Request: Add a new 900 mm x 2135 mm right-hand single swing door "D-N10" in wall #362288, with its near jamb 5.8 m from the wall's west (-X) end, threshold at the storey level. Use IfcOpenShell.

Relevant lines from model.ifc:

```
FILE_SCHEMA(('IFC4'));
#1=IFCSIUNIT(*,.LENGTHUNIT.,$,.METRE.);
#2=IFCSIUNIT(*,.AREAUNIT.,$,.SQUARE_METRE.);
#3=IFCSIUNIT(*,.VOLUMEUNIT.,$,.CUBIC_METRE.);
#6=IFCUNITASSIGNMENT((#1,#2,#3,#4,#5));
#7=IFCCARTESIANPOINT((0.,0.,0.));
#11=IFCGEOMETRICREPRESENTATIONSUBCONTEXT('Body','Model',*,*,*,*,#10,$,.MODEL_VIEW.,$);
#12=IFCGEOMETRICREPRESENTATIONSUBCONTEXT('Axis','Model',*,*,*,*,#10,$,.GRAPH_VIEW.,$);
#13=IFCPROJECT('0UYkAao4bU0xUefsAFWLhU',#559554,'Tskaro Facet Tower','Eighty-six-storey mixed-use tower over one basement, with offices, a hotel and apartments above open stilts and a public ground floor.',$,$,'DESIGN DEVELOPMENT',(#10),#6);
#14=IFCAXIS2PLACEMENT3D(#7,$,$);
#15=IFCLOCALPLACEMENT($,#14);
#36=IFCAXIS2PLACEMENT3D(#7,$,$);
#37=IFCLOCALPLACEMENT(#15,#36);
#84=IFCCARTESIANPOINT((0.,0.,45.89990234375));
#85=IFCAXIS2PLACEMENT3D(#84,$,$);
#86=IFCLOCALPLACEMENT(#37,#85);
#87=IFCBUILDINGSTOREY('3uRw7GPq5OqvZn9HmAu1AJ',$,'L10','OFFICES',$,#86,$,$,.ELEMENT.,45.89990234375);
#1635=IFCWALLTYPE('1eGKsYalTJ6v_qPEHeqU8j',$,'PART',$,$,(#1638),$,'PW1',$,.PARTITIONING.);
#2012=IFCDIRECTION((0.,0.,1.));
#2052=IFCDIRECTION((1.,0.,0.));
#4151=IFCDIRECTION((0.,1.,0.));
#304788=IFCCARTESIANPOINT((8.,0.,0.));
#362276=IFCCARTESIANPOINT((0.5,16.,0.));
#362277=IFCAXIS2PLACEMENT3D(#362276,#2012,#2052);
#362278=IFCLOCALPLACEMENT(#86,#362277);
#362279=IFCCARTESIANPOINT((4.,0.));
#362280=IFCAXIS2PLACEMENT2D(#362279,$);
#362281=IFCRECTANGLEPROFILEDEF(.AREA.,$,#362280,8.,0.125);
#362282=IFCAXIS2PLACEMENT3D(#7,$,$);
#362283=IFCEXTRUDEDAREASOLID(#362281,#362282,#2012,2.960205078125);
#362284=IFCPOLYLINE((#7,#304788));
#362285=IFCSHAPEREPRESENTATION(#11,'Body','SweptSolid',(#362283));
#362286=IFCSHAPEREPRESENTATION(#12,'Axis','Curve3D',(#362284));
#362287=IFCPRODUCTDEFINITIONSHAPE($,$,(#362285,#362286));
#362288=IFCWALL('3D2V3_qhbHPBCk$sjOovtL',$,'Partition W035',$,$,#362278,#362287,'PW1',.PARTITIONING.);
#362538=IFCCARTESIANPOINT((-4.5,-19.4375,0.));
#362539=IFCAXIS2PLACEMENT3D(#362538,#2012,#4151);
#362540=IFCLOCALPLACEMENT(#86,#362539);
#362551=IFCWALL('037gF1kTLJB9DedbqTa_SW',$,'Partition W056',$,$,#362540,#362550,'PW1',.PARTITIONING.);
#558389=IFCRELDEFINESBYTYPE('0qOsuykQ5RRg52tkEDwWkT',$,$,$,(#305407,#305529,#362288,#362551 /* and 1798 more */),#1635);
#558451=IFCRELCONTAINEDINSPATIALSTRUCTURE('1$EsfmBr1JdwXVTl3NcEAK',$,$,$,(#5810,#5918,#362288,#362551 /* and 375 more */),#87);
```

```python
import numpy as np
import ifcopenshell
import ifcopenshell.api.feature
import ifcopenshell.api.geometry
import ifcopenshell.api.root
import ifcopenshell.api.spatial
import ifcopenshell.geom
import ifcopenshell.util.element
import ifcopenshell.util.placement
import ifcopenshell.util.representation
import ifcopenshell.util.shape
import ifcopenshell.util.unit

model = ifcopenshell.open("model.ifc")
unit_scale = ifcopenshell.util.unit.calculate_unit_scale(model)
settings = ifcopenshell.geom.settings()


def volume(element):
    """Net volume in cubic metres, openings subtracted."""
    shape = ifcopenshell.geom.create_shape(settings, element)
    return ifcopenshell.util.shape.get_volume(shape.geometry)


wall = model.by_id(362288)
storey = ifcopenshell.util.element.get_container(wall, ifc_class="IfcBuildingStorey")
context = ifcopenshell.util.representation.get_context(model, "Model", "Body", "MODEL_VIEW")
before = volume(wall)

width, height, from_end, sill = 0.9, 2.135, 5.8, 0.0  # metres

# The wall runs along its own X axis, and the end named is its -X end.
wall_shape = ifcopenshell.geom.create_shape(settings, wall)
x, y, z = ifcopenshell.util.shape.get_vertices(wall_shape.geometry).T
start = x.min() + from_end
face, thickness = float(y.min()), float(y.max() - y.min())
wall_matrix = ifcopenshell.util.placement.get_local_placement(wall.ObjectPlacement)
level = ifcopenshell.util.placement.get_local_placement(storey.ObjectPlacement)[2, 3]


def in_wall(x, y):
    """Placement at x, y metres in the wall's axes, at sill height."""
    matrix = wall_matrix.copy()
    matrix[:, 3] = wall_matrix @ np.array([x / unit_scale, y / unit_scale, 0.0, 1.0])
    matrix[2, 3] = level + sill / unit_scale
    return matrix


# Opening: a box that overshoots both wall faces by 50 mm.
opening = ifcopenshell.api.root.create_entity(model, ifc_class="IfcOpeningElement", predefined_type="OPENING")
box = ifcopenshell.api.geometry.add_wall_representation(
    model, context=context, length=width, height=height, thickness=thickness + 0.1
)
ifcopenshell.api.geometry.assign_representation(model, product=opening, representation=box)
ifcopenshell.api.geometry.edit_object_placement(model, product=opening, matrix=in_wall(start, face - 0.05), is_si=False)
ifcopenshell.api.feature.add_feature(model, feature=opening, element=wall)

door = ifcopenshell.api.root.create_entity(model, ifc_class="IfcDoor", name="D-N10", predefined_type="DOOR")
door.OverallWidth, door.OverallHeight = width / unit_scale, height / unit_scale
door.OperationType = "SINGLE_SWING_RIGHT"
body = ifcopenshell.api.geometry.add_door_representation(
    model,
    context=context,
    overall_width=door.OverallWidth,
    overall_height=door.OverallHeight,
    operation_type="SINGLE_SWING_RIGHT",
    lining_properties={"LiningDepth": thickness / unit_scale, "ThresholdDepth": thickness / unit_scale},
)
ifcopenshell.api.geometry.assign_representation(model, product=door, representation=body)
ifcopenshell.api.spatial.assign_container(model, products=[door], relating_structure=storey)
ifcopenshell.api.feature.add_filling(model, opening=opening, element=door)

# The lining spans the wall, so the door starts at the wall face.
ifcopenshell.api.geometry.edit_object_placement(model, product=door, matrix=in_wall(start, face), is_si=False)

after = volume(wall)

print(f"wall volume {before:.3f} -> {after:.3f} m3")

model.write("model_edited.ifc")
```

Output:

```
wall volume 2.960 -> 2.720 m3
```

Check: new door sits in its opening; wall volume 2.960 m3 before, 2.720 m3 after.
